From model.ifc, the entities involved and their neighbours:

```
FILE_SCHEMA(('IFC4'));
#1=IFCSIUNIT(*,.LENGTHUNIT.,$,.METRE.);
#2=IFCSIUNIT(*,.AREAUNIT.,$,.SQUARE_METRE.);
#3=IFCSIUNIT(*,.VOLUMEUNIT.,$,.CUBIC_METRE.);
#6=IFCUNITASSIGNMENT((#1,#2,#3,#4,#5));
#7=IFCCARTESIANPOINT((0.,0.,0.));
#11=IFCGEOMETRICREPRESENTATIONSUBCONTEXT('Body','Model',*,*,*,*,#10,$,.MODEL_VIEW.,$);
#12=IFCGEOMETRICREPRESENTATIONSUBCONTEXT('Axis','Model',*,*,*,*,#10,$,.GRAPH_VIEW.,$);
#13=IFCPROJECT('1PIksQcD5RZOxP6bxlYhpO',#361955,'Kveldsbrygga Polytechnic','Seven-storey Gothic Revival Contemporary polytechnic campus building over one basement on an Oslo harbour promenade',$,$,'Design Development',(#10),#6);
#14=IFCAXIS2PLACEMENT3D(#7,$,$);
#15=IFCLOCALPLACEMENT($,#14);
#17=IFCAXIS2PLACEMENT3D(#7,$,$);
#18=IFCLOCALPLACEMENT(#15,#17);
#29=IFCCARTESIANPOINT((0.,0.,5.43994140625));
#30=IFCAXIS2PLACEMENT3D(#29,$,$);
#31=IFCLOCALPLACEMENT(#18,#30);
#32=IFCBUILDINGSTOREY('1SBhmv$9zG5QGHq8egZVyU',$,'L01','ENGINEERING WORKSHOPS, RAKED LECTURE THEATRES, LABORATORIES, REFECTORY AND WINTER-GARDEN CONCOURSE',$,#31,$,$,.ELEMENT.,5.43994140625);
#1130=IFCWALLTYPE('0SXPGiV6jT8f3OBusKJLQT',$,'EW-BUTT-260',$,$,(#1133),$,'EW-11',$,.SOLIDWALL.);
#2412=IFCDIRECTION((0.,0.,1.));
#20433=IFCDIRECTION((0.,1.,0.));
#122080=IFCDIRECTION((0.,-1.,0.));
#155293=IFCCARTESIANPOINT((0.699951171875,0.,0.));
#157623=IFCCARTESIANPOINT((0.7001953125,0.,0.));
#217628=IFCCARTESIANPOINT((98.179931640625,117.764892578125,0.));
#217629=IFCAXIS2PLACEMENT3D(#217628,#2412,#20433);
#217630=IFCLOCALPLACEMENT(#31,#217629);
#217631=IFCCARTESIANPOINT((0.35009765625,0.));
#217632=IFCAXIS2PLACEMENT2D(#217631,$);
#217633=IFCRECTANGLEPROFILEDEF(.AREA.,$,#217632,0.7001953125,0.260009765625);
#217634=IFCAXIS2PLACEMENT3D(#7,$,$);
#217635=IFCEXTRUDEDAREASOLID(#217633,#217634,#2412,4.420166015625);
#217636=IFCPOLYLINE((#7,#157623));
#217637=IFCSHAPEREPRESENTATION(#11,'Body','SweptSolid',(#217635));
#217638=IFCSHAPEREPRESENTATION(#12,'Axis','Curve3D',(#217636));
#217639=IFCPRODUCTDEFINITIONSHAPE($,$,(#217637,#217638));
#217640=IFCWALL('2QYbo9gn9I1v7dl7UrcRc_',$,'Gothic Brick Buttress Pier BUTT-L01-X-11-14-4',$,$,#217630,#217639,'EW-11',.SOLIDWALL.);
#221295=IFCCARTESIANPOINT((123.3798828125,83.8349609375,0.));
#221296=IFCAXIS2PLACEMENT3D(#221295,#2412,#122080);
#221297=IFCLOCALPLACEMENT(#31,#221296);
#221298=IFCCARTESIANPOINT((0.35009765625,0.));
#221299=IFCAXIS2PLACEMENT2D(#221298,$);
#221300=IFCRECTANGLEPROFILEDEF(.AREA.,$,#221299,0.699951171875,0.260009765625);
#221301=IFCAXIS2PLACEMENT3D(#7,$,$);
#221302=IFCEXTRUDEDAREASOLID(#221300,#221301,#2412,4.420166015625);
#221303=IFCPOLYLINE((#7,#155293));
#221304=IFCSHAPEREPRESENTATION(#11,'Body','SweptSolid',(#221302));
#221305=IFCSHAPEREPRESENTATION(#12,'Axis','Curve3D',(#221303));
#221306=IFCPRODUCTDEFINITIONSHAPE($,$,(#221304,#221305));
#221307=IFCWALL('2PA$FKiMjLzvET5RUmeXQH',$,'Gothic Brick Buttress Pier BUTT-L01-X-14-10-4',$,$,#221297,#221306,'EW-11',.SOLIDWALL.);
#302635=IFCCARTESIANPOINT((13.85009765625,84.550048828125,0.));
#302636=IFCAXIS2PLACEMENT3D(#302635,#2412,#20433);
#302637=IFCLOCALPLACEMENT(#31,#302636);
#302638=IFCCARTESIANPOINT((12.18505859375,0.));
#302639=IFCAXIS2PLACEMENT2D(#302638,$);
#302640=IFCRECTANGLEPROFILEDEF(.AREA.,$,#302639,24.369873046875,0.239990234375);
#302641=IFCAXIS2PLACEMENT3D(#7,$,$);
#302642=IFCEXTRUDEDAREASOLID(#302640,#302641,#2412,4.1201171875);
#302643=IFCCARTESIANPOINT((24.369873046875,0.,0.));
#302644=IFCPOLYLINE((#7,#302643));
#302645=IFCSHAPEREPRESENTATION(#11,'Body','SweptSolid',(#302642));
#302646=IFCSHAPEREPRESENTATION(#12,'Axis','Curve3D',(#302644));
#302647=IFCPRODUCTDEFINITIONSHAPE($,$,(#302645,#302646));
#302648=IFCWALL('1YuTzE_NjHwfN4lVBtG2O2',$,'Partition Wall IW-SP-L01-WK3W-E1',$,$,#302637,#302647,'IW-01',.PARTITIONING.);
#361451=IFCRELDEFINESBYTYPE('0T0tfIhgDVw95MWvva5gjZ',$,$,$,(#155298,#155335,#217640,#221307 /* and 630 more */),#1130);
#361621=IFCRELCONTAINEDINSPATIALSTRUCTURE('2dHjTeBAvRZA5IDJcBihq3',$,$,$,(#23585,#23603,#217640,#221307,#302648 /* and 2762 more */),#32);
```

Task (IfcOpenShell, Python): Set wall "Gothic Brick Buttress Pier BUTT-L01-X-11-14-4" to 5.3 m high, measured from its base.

```python
import ifcopenshell
import ifcopenshell.geom
import ifcopenshell.util.representation
import ifcopenshell.util.shape

model = ifcopenshell.open("model.ifc")
settings = ifcopenshell.geom.settings()


def volume(element):
    """Net volume in cubic metres, openings subtracted."""
    shape = ifcopenshell.geom.create_shape(settings, element)
    return ifcopenshell.util.shape.get_volume(shape.geometry)


wall = model.by_id(217640)
before = volume(wall)

body = ifcopenshell.util.representation.get_representation(wall, "Model", "Body")
solid = body.Items[0]
old_height = solid.Depth
solid.Depth = 5.3
after = volume(wall)

print(f"height {old_height:g} -> {solid.Depth:g}, volume {before:.3f} -> {after:.3f} m3")

model.write("model_rev.ifc")
```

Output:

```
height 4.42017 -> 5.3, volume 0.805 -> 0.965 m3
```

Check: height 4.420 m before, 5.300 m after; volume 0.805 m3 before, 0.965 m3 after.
